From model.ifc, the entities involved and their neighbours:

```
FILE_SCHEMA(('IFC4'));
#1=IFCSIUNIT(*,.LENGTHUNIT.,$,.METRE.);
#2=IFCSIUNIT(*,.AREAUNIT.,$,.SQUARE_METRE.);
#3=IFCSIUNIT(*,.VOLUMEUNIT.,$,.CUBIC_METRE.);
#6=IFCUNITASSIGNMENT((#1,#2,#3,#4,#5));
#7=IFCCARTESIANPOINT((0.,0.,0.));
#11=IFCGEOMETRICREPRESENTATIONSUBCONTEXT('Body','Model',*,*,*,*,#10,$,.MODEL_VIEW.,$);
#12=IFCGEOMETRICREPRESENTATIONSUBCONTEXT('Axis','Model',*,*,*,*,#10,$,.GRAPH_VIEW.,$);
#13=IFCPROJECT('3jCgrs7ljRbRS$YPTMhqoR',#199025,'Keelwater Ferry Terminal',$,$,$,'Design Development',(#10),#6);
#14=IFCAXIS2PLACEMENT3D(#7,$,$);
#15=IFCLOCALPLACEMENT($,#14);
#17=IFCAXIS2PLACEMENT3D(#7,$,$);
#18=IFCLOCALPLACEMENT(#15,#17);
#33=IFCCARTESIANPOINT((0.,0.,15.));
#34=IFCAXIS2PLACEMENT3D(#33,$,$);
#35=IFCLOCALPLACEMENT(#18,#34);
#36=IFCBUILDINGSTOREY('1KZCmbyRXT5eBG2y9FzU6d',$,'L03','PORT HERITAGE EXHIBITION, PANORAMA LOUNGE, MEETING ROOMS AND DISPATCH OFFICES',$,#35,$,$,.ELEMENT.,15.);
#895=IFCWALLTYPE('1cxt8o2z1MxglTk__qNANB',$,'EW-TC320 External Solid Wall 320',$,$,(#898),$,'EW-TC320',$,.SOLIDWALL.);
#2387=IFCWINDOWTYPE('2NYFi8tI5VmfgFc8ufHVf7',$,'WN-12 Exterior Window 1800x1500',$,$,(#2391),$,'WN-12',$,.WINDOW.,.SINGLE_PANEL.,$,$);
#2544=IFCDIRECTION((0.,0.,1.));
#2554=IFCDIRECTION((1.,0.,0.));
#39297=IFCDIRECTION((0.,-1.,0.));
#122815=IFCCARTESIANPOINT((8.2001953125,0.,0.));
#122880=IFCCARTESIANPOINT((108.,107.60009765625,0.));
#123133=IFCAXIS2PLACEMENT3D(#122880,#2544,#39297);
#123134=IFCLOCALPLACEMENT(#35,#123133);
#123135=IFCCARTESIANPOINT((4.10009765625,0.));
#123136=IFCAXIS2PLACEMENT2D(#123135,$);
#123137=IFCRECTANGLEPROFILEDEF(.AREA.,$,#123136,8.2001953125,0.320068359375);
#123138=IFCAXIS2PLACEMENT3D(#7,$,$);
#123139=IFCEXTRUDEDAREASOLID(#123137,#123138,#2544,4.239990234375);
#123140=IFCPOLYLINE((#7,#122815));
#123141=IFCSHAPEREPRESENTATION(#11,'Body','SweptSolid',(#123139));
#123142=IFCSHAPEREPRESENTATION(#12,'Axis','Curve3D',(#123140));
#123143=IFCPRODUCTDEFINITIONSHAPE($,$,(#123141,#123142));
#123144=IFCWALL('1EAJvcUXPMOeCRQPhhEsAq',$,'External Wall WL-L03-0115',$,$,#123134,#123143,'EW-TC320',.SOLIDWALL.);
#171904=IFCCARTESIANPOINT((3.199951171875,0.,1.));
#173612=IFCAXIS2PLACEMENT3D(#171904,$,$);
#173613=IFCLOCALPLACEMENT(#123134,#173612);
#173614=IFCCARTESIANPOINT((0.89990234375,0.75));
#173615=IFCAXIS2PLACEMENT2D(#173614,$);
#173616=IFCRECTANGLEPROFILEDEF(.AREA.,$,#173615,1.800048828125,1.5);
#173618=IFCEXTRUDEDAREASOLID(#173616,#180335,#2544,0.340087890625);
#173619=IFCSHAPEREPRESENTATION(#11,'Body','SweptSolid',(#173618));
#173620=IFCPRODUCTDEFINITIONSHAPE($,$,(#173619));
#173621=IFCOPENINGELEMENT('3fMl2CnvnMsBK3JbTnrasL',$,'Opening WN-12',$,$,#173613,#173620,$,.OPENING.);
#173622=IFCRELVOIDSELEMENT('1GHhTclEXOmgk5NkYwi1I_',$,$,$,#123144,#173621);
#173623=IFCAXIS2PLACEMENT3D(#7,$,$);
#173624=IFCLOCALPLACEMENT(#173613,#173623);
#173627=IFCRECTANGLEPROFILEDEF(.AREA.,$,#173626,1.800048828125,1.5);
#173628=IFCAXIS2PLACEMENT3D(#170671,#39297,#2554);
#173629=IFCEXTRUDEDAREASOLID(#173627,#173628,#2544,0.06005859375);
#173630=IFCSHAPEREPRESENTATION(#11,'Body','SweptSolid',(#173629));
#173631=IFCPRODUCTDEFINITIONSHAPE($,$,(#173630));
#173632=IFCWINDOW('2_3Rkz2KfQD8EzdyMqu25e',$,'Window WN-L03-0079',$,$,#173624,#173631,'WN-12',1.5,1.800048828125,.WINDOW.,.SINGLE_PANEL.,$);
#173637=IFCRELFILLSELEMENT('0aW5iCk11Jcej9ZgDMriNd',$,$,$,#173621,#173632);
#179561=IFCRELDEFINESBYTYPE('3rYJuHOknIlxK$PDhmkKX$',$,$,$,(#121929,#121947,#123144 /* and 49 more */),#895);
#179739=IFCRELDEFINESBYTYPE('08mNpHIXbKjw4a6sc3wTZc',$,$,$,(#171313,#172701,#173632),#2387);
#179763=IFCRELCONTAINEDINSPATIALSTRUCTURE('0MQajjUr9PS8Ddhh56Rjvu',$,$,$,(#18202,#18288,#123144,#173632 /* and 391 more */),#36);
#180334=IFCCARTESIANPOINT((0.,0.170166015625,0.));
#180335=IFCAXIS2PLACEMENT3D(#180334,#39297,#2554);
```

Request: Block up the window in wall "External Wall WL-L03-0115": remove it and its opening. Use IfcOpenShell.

```python
import ifcopenshell
import ifcopenshell.api.feature
import ifcopenshell.api.root
import ifcopenshell.geom
import ifcopenshell.util.shape

model = ifcopenshell.open("model.ifc")
settings = ifcopenshell.geom.settings()


def volume(element):
    """Net volume in cubic metres, openings subtracted."""
    shape = ifcopenshell.geom.create_shape(settings, element)
    return ifcopenshell.util.shape.get_volume(shape.geometry)


window = model.by_guid("2_3Rkz2KfQD8EzdyMqu25e")
opening = window.FillsVoids[0].RelatingOpeningElement
wall = opening.VoidsElements[0].RelatingBuildingElement
before = volume(wall)

ifcopenshell.api.root.remove_product(model, product=window)
ifcopenshell.api.feature.remove_feature(model, feature=opening)

after = volume(wall)

print(f"wall volume {before:.3f} -> {after:.3f} m3")

model.write("model_rev.ifc")
```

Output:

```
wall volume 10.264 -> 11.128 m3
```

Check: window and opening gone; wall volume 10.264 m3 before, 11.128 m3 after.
